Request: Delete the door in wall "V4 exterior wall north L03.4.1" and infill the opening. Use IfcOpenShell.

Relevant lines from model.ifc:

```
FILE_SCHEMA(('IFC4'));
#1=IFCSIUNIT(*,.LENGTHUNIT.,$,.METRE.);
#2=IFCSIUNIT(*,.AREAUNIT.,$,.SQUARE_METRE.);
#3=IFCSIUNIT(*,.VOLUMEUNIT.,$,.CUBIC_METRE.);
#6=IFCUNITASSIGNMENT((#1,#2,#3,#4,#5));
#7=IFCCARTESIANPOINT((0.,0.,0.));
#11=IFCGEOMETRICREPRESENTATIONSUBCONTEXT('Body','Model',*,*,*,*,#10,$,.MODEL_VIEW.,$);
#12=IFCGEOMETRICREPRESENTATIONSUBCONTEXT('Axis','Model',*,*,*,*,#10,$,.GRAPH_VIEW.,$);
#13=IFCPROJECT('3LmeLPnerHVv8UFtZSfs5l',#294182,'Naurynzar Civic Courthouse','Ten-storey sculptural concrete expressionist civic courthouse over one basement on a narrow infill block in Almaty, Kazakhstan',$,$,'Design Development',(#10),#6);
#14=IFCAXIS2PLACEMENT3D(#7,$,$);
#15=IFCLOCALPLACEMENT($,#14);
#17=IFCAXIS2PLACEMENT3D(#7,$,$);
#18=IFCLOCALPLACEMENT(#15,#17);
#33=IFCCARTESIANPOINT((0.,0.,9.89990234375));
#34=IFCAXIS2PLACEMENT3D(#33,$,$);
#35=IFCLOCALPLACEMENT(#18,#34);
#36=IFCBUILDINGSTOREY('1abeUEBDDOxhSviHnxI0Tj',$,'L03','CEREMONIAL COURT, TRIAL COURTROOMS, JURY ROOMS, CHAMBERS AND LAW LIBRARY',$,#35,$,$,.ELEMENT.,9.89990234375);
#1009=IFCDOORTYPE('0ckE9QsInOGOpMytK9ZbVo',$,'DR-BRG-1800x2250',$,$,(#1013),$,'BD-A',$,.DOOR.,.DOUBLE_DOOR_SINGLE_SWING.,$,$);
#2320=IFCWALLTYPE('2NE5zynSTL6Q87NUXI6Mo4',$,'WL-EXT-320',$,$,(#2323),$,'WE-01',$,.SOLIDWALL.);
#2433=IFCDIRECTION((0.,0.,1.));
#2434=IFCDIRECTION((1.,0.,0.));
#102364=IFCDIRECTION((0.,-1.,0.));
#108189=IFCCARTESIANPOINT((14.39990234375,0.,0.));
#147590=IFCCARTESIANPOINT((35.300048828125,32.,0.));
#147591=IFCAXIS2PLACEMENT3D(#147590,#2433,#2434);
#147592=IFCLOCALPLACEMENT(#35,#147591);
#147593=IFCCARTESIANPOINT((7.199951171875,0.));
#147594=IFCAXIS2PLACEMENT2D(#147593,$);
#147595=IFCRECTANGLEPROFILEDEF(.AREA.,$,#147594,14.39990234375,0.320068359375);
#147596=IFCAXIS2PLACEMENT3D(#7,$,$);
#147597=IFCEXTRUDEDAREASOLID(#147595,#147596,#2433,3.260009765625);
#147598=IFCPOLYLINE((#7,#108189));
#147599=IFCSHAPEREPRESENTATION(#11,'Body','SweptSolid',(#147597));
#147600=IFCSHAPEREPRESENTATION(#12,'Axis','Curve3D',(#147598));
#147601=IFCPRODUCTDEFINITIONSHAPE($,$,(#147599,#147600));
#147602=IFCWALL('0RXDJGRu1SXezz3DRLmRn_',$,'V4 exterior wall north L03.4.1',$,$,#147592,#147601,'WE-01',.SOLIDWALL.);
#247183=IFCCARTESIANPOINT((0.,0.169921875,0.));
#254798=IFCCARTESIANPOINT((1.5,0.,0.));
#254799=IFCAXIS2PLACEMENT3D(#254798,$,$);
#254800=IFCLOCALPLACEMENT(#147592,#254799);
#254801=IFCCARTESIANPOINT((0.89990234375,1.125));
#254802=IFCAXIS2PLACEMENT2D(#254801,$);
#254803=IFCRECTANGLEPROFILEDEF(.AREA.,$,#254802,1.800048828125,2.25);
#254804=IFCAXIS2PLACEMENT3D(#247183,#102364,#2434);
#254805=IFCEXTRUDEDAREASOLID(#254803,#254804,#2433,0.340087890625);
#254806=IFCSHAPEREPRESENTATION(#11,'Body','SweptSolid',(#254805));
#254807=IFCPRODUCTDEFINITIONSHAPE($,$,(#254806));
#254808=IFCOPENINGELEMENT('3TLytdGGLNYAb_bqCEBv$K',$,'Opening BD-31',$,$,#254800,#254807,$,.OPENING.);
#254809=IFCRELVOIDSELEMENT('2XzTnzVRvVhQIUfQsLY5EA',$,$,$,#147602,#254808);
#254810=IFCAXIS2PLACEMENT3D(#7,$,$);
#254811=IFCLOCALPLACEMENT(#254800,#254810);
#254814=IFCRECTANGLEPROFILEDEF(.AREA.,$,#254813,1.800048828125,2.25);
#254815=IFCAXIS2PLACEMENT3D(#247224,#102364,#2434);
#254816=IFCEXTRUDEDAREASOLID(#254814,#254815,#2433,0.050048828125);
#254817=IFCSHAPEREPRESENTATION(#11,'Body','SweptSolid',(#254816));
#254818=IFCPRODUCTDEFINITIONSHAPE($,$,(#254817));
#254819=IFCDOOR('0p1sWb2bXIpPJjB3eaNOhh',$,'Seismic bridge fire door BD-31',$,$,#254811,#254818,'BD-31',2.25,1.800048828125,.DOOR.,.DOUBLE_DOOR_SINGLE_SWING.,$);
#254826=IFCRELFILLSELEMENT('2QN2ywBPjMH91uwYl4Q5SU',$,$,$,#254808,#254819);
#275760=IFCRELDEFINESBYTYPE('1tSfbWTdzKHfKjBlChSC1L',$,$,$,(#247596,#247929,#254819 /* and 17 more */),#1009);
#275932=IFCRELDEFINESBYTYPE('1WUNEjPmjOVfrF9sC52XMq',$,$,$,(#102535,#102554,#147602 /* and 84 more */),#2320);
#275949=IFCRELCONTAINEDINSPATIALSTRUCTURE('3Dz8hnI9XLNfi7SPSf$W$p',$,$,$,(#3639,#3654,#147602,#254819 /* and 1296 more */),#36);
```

```python
import ifcopenshell
import ifcopenshell.api.feature
import ifcopenshell.api.root
import ifcopenshell.geom
import ifcopenshell.util.shape

model = ifcopenshell.open("model.ifc")
settings = ifcopenshell.geom.settings()


def volume(element):
    """Net volume in cubic metres, openings subtracted."""
    shape = ifcopenshell.geom.create_shape(settings, element)
    return ifcopenshell.util.shape.get_volume(shape.geometry)


door = model.by_guid("0p1sWb2bXIpPJjB3eaNOhh")
opening = door.FillsVoids[0].RelatingOpeningElement
wall = opening.VoidsElements[0].RelatingBuildingElement
before = volume(wall)

ifcopenshell.api.root.remove_product(model, product=door)
ifcopenshell.api.feature.remove_feature(model, feature=opening)

after = volume(wall)

print(f"wall volume {before:.3f} -> {after:.3f} m3")

model.write("model_rev.ifc")
```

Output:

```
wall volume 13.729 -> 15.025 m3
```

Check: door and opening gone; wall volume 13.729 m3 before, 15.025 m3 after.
